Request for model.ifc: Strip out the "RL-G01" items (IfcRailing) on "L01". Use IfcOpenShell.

First a look at what the model holds.

```python
import ifcopenshell
import ifcopenshell.util.element

model = ifcopenshell.open("model.ifc")
print(model.schema)
storey = next(s for s in model.by_type("IfcBuildingStorey") if s.Name == "L01")
railings = [e for e in ifcopenshell.util.element.get_decomposition(storey) if e.is_a("IfcRailing")]
seen = {}
for e in railings:
    element_type = ifcopenshell.util.element.get_type(e)
    name = element_type.Name if element_type not in (None, e) else None
    seen[name] = seen.get(name, 0) + 1
for name, count in sorted(seen.items(), key=str):
    print(count, "x", name)
```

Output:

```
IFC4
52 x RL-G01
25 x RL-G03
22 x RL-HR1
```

```python
import ifcopenshell
import ifcopenshell.api.root
import ifcopenshell.util.element

model = ifcopenshell.open("model.ifc")

storey = next(s for s in model.by_type("IfcBuildingStorey") if s.Name == "L01")
railings = [e for e in ifcopenshell.util.element.get_decomposition(storey) if e.is_a("IfcRailing")]
targets = [e for e in railings if (t := ifcopenshell.util.element.get_type(e)) not in (None, e) and t.Name == "RL-G01"]

for e in targets:
    ifcopenshell.api.root.remove_product(model, product=e)
print(len(targets), "removed")

model.write("model-out.ifc")
```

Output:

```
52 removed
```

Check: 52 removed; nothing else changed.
